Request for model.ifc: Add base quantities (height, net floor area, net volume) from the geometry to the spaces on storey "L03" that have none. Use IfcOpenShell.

First a look at what the model holds.

```python
import ifcopenshell
import ifcopenshell.util.element
import ifcopenshell.util.unit

model = ifcopenshell.open("model.ifc")
print(model.schema)
for unit_type in ("LENGTHUNIT", "AREAUNIT", "VOLUMEUNIT"):
    print(unit_type, ifcopenshell.util.unit.calculate_unit_scale(model, unit_type))
storey = next(s for s in model.by_type("IfcBuildingStorey") if s.Name == "L03")
spaces = [e for e in ifcopenshell.util.element.get_decomposition(storey) if e.is_a("IfcSpace")]
for e in sorted(spaces, key=lambda e: e.id()):
    print(e.id(), e.is_a(), e.Name, list(ifcopenshell.util.element.get_psets(e, qtos_only=True)), sep=" | ")
```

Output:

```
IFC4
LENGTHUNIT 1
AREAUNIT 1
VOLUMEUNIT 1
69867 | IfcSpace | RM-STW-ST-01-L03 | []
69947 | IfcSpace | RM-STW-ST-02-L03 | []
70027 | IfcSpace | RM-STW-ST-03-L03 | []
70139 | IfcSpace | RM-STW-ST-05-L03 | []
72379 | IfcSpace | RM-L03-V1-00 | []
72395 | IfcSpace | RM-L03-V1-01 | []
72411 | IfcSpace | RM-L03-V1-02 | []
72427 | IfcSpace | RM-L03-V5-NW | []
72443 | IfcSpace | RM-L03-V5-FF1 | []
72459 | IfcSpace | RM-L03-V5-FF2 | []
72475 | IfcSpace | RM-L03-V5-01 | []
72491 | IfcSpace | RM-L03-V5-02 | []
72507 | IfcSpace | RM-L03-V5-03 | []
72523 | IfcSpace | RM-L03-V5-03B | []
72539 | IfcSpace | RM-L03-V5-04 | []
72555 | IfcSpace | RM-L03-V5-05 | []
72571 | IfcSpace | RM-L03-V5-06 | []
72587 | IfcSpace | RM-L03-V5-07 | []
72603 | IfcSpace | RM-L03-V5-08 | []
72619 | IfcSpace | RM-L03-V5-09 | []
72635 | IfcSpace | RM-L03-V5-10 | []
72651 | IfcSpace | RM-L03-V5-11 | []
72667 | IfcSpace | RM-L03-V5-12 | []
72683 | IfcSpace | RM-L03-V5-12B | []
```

```python
import ifcopenshell
import ifcopenshell.api.pset
import ifcopenshell.geom
import ifcopenshell.util.element
import ifcopenshell.util.shape
import ifcopenshell.util.unit

model = ifcopenshell.open("model.ifc")
unit_scale = ifcopenshell.util.unit.calculate_unit_scale(model)
area_scale = ifcopenshell.util.unit.calculate_unit_scale(model, "AREAUNIT")
volume_scale = ifcopenshell.util.unit.calculate_unit_scale(model, "VOLUMEUNIT")
settings = ifcopenshell.geom.settings()

storey = next(s for s in model.by_type("IfcBuildingStorey") if s.Name == "L03")
spaces = [e for e in ifcopenshell.util.element.get_decomposition(storey) if e.is_a("IfcSpace")]

for e in sorted(spaces, key=lambda e: e.id()):
    if ifcopenshell.util.element.get_psets(e, qtos_only=True, should_inherit=False):
        continue
    # Geometry comes back in metres, in the element's own axes.
    shape = ifcopenshell.geom.create_shape(settings, e)
    values = {
        "Height": ifcopenshell.util.shape.get_z(shape.geometry) / unit_scale,
        "NetFloorArea": ifcopenshell.util.shape.get_footprint_area(shape.geometry) / area_scale,
        "NetVolume": ifcopenshell.util.shape.get_volume(shape.geometry) / volume_scale,
    }
    qto = ifcopenshell.api.pset.add_qto(model, product=e, name="Qto_SpaceBaseQuantities")
    ifcopenshell.api.pset.edit_qto(model, qto=qto, properties=values)
    print(e.id(), {k: round(v, 3) for k, v in values.items()})

model.write("model-out.ifc")
```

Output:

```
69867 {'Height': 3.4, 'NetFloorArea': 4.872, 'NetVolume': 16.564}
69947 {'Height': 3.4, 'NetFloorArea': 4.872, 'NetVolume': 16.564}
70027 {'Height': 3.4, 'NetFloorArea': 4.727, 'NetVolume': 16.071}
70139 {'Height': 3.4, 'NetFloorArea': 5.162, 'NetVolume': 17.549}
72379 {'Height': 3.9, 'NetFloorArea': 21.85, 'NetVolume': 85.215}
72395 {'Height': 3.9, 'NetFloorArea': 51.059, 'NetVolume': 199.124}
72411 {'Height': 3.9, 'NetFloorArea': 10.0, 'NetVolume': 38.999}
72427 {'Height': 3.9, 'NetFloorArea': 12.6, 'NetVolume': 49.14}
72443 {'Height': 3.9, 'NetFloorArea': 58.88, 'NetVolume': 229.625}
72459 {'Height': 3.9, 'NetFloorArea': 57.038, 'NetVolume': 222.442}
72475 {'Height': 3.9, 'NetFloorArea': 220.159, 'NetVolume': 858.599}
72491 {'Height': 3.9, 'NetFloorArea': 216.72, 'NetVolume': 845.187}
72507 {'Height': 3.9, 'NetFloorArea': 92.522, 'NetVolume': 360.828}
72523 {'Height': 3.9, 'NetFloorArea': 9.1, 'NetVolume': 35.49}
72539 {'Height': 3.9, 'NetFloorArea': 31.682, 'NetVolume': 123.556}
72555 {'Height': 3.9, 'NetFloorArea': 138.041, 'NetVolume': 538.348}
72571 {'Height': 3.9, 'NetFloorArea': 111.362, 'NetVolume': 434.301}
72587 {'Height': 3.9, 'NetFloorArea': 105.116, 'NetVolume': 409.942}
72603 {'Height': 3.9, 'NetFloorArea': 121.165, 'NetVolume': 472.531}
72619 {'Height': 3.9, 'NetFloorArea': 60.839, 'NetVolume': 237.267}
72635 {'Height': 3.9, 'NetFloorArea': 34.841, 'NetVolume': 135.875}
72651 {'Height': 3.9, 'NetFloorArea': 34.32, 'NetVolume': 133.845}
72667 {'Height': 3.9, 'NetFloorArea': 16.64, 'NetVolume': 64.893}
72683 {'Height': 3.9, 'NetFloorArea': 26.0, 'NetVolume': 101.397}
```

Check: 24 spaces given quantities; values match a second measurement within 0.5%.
